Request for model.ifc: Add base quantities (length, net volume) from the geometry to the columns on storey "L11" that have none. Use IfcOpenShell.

First a look at what the model holds.

```python
import ifcopenshell
import ifcopenshell.util.element
import ifcopenshell.util.unit

model = ifcopenshell.open("model.ifc")
print(model.schema)
for unit_type in ("LENGTHUNIT", "AREAUNIT", "VOLUMEUNIT"):
    print(unit_type, ifcopenshell.util.unit.calculate_unit_scale(model, unit_type))
storey = next(s for s in model.by_type("IfcBuildingStorey") if s.Name == "L11")
columns = [e for e in ifcopenshell.util.element.get_decomposition(storey) if e.is_a("IfcColumn")]
for e in sorted(columns, key=lambda e: e.id()):
    print(e.id(), e.is_a(), e.Name, list(ifcopenshell.util.element.get_psets(e, qtos_only=True)), sep=" | ")
```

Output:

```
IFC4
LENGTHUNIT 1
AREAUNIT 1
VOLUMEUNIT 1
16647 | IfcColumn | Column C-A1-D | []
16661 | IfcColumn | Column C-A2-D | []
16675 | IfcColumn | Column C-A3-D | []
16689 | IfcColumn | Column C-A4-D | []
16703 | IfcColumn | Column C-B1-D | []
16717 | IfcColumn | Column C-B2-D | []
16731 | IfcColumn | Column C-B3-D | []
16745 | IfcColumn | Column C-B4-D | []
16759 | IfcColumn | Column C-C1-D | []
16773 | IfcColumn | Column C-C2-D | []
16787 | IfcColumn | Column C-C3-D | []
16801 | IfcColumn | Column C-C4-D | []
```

```python
import ifcopenshell
import ifcopenshell.api.pset
import ifcopenshell.geom
import ifcopenshell.util.element
import ifcopenshell.util.shape
import ifcopenshell.util.unit

model = ifcopenshell.open("model.ifc")
unit_scale = ifcopenshell.util.unit.calculate_unit_scale(model)
volume_scale = ifcopenshell.util.unit.calculate_unit_scale(model, "VOLUMEUNIT")
settings = ifcopenshell.geom.settings()

storey = next(s for s in model.by_type("IfcBuildingStorey") if s.Name == "L11")
columns = [e for e in ifcopenshell.util.element.get_decomposition(storey) if e.is_a("IfcColumn")]

for e in sorted(columns, key=lambda e: e.id()):
    if ifcopenshell.util.element.get_psets(e, qtos_only=True, should_inherit=False):
        continue
    # Geometry comes back in metres, in the element's own axes.
    shape = ifcopenshell.geom.create_shape(settings, e)
    values = {
        "Length": ifcopenshell.util.shape.get_z(shape.geometry) / unit_scale,
        "NetVolume": ifcopenshell.util.shape.get_volume(shape.geometry) / volume_scale,
    }
    qto = ifcopenshell.api.pset.add_qto(model, product=e, name="Qto_ColumnBaseQuantities")
    ifcopenshell.api.pset.edit_qto(model, qto=qto, properties=values)
    print(e.id(), {k: round(v, 3) for k, v in values.items()})

model.write("model_updated.ifc")
```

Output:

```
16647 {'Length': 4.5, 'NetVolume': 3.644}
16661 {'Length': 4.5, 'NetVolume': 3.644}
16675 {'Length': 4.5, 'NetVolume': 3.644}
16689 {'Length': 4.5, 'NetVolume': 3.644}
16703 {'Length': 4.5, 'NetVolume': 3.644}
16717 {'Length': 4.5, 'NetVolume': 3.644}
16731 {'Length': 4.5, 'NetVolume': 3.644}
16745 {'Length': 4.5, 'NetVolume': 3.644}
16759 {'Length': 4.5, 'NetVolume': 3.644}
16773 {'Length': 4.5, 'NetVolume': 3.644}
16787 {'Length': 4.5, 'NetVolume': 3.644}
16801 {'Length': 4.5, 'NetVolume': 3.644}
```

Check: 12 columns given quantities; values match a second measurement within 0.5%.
